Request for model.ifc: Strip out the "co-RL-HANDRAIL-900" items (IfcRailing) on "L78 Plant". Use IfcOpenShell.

First a look at what the model holds.

```python
import ifcopenshell
import ifcopenshell.util.element

model = ifcopenshell.open("model.ifc")
print(model.schema)
storey = next(s for s in model.by_type("IfcBuildingStorey") if s.Name == "L78 Plant")
railings = [e for e in ifcopenshell.util.element.get_decomposition(storey) if e.is_a("IfcRailing")]
seen = {}
for e in railings:
    element_type = ifcopenshell.util.element.get_type(e)
    name = element_type.Name if element_type not in (None, e) else None
    seen[name] = seen.get(name, 0) + 1
for name, count in sorted(seen.items(), key=str):
    print(count, "x", name)
```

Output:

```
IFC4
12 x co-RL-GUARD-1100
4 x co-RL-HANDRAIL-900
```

```python
import ifcopenshell
import ifcopenshell.api.root
import ifcopenshell.util.element

model = ifcopenshell.open("model.ifc")

storey = next(s for s in model.by_type("IfcBuildingStorey") if s.Name == "L78 Plant")
railings = [e for e in ifcopenshell.util.element.get_decomposition(storey) if e.is_a("IfcRailing")]
targets = [e for e in railings if (t := ifcopenshell.util.element.get_type(e)) not in (None, e) and t.Name == "co-RL-HANDRAIL-900"]

for e in targets:
    ifcopenshell.api.root.remove_product(model, product=e)
print(len(targets), "removed")

model.write("model-out.ifc")
```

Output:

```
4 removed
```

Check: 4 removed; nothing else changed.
